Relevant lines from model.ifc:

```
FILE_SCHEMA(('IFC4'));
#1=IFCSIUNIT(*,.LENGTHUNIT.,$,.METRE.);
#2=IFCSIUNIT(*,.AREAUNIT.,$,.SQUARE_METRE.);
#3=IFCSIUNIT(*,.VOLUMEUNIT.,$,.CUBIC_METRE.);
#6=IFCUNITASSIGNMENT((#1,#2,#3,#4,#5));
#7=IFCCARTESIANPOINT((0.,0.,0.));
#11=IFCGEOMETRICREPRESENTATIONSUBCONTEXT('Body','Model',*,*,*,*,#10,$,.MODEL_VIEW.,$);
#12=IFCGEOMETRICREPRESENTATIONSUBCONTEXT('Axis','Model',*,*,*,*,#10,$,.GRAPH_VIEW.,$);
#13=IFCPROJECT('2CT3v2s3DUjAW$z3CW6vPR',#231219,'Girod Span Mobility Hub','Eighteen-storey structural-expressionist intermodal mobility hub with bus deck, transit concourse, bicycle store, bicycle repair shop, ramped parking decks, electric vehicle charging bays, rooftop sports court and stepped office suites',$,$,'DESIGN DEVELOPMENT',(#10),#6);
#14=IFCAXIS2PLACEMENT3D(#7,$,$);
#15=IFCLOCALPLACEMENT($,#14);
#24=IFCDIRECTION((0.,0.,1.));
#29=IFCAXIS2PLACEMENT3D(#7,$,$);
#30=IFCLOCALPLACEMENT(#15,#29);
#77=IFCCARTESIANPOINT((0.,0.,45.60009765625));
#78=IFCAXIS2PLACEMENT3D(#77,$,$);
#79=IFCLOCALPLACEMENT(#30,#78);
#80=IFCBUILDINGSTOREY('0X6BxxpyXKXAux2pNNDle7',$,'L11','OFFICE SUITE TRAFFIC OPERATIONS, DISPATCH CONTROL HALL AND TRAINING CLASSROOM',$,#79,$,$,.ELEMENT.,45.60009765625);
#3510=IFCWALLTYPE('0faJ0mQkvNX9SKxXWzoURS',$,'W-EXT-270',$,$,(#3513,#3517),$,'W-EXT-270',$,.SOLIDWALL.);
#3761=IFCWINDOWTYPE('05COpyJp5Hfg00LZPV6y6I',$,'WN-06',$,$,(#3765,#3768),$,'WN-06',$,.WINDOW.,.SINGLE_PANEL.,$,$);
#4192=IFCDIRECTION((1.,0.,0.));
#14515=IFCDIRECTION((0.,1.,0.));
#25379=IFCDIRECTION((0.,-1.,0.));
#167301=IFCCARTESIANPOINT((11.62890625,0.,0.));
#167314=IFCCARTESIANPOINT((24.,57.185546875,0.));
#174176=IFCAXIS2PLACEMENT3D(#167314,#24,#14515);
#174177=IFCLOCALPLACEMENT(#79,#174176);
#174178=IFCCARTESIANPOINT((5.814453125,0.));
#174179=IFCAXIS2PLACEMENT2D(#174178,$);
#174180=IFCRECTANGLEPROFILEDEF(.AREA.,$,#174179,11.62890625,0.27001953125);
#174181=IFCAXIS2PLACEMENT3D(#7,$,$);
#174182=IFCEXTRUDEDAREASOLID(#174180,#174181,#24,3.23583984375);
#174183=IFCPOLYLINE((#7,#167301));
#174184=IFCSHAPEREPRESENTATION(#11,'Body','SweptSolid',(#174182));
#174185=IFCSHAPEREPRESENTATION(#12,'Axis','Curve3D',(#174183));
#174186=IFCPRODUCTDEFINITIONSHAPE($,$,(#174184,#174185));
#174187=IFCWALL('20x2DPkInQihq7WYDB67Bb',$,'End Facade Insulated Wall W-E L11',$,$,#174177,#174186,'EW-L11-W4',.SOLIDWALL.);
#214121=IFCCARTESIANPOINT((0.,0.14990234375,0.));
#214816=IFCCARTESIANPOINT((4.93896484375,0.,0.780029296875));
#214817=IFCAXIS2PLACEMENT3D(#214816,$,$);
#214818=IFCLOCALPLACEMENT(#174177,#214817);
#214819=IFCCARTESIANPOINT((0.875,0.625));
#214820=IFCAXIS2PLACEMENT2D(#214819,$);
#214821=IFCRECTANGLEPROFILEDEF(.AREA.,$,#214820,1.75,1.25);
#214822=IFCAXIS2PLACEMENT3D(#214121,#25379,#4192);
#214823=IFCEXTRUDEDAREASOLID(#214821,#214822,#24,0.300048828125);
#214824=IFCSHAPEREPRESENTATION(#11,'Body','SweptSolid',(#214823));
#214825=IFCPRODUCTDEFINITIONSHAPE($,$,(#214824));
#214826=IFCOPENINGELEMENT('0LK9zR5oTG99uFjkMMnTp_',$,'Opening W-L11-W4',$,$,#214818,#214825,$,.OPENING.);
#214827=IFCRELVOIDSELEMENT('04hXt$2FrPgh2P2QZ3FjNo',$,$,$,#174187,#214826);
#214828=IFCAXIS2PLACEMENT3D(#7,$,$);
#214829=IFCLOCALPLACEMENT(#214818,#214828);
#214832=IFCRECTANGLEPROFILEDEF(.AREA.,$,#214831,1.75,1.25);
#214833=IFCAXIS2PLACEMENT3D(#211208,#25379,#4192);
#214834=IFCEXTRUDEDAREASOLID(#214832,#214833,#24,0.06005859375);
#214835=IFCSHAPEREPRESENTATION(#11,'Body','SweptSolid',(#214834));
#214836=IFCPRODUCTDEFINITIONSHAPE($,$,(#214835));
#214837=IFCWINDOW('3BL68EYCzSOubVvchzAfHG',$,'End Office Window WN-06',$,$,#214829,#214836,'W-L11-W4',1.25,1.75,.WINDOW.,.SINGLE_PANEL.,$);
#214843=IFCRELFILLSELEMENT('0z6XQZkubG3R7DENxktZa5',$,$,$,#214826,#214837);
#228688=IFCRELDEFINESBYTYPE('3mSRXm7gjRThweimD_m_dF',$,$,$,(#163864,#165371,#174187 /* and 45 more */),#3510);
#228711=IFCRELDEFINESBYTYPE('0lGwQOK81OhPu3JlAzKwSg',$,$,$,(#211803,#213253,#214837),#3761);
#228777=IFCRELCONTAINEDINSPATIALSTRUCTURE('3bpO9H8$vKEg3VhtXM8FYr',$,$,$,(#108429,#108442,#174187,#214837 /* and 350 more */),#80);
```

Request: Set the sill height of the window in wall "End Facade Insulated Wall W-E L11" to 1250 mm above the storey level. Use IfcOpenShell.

```python
import numpy as np
import ifcopenshell
import ifcopenshell.api.geometry
import ifcopenshell.geom
import ifcopenshell.util.element
import ifcopenshell.util.placement
import ifcopenshell.util.shape
import ifcopenshell.util.unit

model = ifcopenshell.open("model.ifc")
unit_scale = ifcopenshell.util.unit.calculate_unit_scale(model)

window = model.by_guid("3BL68EYCzSOubVvchzAfHG")
opening = window.FillsVoids[0].RelatingOpeningElement
storey = ifcopenshell.util.element.get_container(window, ifc_class="IfcBuildingStorey")
level = ifcopenshell.util.placement.get_local_placement(storey.ObjectPlacement)[2, 3]

# The opening's origin need not be at the sill, so measure its lowest point.
shape = ifcopenshell.geom.create_shape(ifcopenshell.geom.settings(), opening)
bottom = ifcopenshell.util.shape.get_shape_bottom_elevation(shape, shape.geometry) / unit_scale
dz = level + 1.25 / unit_scale - bottom

shift = np.array([0.0, 0.0, dz])
# The window is placed relative to its opening, so it follows when the opening moves.
matrix = ifcopenshell.util.placement.get_local_placement(opening.ObjectPlacement)
matrix[:3, 3] += shift
ifcopenshell.api.geometry.edit_object_placement(
    model, product=opening, matrix=matrix, is_si=False, should_transform_children=True
)

print(f"moved by {dz * unit_scale:+.3f} m")

model.write("model_edited.ifc")
```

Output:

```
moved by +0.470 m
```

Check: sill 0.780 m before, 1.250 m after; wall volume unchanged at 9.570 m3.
